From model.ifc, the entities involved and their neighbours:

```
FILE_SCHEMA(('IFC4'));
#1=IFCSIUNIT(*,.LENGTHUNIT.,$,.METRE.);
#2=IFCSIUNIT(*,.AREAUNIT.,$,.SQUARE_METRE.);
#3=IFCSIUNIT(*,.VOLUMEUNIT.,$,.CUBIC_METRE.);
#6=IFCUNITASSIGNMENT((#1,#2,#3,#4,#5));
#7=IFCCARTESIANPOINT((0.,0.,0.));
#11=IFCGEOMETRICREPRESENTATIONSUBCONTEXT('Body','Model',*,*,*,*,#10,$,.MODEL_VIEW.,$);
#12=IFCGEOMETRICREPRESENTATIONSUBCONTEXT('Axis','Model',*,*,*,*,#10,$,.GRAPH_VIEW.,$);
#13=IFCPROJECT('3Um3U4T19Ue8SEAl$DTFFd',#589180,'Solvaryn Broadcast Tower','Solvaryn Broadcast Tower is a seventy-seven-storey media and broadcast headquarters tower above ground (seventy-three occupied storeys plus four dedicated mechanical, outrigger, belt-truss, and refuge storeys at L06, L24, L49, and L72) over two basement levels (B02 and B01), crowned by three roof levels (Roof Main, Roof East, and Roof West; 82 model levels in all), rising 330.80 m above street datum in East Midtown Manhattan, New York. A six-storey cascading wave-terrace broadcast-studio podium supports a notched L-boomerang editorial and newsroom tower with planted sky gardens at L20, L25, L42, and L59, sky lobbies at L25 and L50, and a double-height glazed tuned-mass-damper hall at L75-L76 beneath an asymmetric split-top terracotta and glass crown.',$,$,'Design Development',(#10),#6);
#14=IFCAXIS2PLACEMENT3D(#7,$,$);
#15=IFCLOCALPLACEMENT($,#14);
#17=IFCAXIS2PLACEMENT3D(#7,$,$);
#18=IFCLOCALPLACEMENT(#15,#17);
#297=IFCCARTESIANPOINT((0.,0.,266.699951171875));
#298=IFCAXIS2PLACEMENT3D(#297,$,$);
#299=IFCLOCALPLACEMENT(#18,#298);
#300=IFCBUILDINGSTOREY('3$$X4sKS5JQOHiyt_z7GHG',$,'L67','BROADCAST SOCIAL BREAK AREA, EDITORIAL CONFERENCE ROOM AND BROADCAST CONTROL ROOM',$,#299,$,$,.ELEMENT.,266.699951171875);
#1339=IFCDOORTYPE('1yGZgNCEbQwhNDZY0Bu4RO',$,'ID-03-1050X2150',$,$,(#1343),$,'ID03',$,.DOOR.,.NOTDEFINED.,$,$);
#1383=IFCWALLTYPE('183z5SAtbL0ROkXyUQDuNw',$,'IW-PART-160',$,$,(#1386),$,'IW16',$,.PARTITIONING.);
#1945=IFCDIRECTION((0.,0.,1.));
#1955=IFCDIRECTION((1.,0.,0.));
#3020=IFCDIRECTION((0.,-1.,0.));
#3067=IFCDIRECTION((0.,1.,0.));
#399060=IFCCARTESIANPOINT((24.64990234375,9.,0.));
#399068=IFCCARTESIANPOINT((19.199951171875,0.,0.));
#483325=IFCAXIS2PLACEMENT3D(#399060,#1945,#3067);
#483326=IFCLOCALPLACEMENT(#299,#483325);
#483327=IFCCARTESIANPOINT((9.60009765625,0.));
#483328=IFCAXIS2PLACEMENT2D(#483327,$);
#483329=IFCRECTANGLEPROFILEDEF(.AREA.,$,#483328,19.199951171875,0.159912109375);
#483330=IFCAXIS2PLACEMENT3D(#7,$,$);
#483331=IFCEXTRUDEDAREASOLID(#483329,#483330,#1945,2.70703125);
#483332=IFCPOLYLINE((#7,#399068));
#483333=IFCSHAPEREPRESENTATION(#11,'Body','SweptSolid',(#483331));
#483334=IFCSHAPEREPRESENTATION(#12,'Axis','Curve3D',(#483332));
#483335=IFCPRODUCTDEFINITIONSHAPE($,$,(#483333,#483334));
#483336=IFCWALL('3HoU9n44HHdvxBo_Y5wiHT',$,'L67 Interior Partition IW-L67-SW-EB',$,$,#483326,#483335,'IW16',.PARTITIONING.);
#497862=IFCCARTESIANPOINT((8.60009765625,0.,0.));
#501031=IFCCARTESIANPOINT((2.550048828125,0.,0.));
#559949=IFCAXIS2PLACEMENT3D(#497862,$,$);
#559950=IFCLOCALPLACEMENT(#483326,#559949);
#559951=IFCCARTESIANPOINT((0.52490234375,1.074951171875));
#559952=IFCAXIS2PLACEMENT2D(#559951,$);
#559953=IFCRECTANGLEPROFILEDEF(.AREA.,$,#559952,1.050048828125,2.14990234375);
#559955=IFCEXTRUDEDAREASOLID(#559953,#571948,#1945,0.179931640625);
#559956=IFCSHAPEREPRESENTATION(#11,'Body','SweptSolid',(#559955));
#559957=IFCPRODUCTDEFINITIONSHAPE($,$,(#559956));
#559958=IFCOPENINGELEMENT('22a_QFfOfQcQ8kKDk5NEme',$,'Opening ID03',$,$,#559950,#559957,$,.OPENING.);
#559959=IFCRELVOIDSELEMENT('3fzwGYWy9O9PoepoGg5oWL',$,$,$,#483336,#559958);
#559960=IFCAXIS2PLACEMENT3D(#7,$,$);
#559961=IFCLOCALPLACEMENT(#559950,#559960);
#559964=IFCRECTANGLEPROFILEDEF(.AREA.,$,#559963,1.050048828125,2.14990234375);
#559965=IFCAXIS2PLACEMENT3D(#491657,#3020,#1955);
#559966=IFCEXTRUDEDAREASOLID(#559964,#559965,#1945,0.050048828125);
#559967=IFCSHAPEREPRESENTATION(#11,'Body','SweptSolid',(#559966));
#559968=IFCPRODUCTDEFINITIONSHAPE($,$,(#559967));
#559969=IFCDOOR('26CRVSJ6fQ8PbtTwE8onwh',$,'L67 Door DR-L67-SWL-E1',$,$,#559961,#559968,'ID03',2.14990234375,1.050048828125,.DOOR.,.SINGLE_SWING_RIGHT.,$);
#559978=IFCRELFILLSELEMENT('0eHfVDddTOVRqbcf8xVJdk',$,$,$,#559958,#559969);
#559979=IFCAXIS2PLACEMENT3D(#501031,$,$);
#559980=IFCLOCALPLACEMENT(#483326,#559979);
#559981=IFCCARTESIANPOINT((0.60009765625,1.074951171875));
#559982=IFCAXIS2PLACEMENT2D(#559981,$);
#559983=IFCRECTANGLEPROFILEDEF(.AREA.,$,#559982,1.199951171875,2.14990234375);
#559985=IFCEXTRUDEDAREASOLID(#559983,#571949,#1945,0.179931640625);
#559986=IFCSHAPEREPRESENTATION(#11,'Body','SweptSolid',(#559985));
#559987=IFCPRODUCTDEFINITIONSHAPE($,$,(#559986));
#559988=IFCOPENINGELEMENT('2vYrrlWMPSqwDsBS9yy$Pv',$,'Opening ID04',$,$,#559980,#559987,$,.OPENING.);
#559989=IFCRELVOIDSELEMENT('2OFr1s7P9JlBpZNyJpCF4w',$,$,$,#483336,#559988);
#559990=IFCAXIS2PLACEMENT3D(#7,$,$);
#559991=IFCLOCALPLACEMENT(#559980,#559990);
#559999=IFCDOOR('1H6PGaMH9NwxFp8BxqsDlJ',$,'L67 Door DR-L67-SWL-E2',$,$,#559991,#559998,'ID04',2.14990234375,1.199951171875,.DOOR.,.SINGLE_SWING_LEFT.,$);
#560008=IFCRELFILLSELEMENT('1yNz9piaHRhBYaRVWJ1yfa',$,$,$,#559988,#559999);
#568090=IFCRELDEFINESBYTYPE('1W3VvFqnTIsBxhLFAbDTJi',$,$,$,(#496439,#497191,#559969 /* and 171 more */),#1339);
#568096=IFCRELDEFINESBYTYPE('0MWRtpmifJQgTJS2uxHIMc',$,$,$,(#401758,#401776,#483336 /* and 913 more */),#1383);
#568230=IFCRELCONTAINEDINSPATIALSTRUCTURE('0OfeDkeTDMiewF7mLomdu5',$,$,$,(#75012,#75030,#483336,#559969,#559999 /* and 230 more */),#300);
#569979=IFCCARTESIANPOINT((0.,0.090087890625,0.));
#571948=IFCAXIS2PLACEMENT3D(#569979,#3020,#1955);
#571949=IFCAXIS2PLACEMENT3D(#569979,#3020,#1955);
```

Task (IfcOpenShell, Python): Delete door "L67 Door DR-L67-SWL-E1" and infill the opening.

```python
import ifcopenshell
import ifcopenshell.api.feature
import ifcopenshell.api.root
import ifcopenshell.geom
import ifcopenshell.util.shape

model = ifcopenshell.open("model.ifc")
settings = ifcopenshell.geom.settings()


def volume(element):
    """Net volume in cubic metres, openings subtracted."""
    shape = ifcopenshell.geom.create_shape(settings, element)
    return ifcopenshell.util.shape.get_volume(shape.geometry)


door = model.by_id(559969)
opening = door.FillsVoids[0].RelatingOpeningElement
wall = opening.VoidsElements[0].RelatingBuildingElement
before = volume(wall)

ifcopenshell.api.root.remove_product(model, product=door)
ifcopenshell.api.feature.remove_feature(model, feature=opening)

after = volume(wall)

print(f"wall volume {before:.3f} -> {after:.3f} m3")

model.write("model_edited.ifc")
```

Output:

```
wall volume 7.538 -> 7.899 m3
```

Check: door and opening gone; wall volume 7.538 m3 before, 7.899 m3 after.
